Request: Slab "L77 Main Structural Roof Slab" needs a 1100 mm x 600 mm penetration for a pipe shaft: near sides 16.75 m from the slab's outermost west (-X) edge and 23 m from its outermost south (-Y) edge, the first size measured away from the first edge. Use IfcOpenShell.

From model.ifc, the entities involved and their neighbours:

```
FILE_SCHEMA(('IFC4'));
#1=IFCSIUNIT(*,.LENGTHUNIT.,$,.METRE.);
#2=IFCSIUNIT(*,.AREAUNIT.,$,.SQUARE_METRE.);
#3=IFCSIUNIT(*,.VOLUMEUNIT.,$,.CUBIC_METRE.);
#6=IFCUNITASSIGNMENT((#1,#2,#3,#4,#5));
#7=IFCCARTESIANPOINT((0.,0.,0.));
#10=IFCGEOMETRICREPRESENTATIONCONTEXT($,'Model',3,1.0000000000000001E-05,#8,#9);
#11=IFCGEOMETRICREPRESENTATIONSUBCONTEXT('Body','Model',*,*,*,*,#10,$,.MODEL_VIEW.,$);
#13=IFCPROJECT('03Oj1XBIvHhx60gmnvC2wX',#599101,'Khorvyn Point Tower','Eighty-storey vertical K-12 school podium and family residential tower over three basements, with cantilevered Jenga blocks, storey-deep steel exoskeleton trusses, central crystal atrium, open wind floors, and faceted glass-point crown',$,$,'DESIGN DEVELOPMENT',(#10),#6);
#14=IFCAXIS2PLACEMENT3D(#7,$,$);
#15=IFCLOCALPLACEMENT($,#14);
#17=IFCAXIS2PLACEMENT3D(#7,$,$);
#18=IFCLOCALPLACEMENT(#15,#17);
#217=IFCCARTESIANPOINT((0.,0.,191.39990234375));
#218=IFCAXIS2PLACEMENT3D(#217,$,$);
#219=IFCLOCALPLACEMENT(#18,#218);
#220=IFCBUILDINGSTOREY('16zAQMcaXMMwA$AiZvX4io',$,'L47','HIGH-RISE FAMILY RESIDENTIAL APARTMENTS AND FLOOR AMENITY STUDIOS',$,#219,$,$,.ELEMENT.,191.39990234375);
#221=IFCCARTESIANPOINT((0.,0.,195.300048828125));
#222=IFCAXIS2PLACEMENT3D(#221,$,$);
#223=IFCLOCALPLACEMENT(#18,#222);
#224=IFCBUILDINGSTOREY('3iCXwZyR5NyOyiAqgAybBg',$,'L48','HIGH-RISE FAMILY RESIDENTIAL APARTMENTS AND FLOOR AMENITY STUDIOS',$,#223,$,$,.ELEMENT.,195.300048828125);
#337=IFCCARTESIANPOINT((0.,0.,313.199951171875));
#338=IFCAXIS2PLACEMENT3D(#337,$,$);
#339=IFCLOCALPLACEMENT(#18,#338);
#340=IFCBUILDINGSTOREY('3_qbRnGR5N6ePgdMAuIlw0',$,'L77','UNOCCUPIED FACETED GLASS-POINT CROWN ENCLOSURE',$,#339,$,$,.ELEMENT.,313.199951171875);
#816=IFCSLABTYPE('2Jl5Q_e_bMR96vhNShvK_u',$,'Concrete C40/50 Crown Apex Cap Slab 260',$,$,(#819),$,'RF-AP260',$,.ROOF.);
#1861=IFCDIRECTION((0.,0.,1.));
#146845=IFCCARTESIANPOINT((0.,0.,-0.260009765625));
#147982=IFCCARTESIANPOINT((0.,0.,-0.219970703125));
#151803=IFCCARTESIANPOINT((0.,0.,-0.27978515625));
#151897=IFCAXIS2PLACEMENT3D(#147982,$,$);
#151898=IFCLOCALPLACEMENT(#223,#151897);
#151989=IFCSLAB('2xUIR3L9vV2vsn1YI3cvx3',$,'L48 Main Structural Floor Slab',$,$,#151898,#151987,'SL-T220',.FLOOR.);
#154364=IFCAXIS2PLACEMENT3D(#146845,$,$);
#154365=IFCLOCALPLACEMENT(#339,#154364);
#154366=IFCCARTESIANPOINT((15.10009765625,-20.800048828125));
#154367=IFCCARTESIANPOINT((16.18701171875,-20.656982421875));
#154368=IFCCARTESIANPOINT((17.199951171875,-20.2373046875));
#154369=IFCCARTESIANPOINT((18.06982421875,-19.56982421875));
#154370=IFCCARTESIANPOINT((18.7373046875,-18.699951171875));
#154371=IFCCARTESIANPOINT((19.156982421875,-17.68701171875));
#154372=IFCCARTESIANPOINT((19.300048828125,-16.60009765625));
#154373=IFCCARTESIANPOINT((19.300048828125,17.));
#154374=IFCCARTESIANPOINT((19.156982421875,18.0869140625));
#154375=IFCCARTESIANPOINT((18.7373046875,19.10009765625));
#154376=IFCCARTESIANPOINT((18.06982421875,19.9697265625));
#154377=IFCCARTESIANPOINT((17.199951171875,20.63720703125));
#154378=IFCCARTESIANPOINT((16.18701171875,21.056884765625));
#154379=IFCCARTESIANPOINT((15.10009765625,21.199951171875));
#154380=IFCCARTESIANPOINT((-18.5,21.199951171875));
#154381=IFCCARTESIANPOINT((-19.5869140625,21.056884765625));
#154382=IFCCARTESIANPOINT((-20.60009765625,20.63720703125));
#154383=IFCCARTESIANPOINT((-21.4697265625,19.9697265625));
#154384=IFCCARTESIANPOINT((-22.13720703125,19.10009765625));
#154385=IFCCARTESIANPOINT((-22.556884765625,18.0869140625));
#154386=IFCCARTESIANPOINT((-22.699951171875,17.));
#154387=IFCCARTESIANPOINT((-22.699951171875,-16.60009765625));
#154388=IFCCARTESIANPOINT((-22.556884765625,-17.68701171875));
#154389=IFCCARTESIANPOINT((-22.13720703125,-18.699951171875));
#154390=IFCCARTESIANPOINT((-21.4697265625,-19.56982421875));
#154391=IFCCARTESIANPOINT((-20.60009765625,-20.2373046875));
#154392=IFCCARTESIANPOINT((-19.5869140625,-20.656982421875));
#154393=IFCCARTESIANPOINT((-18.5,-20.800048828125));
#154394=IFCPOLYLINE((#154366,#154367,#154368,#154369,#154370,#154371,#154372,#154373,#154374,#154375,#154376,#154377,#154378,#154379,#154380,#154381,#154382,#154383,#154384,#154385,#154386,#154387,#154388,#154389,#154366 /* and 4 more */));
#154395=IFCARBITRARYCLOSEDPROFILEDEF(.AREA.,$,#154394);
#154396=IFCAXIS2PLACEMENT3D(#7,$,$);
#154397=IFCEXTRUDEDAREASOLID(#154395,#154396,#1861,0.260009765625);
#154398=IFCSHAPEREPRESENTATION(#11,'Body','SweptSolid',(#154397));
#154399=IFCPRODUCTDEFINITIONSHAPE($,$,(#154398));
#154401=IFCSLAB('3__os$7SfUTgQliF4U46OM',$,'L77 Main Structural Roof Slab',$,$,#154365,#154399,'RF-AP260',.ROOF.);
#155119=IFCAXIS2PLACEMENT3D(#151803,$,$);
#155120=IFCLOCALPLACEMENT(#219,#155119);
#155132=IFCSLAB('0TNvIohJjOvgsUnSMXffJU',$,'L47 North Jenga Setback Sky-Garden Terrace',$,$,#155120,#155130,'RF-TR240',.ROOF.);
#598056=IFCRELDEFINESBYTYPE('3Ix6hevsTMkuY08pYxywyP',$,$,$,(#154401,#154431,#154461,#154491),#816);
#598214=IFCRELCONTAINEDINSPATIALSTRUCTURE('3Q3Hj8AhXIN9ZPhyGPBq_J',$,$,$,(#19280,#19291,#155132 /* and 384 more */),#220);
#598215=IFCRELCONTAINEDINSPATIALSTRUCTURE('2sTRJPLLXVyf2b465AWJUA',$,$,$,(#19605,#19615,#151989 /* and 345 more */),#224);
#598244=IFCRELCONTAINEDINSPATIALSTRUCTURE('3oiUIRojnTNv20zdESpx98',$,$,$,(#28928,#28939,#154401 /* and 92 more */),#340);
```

```python
import numpy as np
import ifcopenshell
import ifcopenshell.api.feature
import ifcopenshell.api.geometry
import ifcopenshell.api.root
import ifcopenshell.geom
import ifcopenshell.util.placement
import ifcopenshell.util.representation
import ifcopenshell.util.shape
import ifcopenshell.util.unit

model = ifcopenshell.open("model.ifc")
unit_scale = ifcopenshell.util.unit.calculate_unit_scale(model)
settings = ifcopenshell.geom.settings()


def volume(element):
    """Net volume in cubic metres, openings subtracted."""
    shape = ifcopenshell.geom.create_shape(settings, element)
    return ifcopenshell.util.shape.get_volume(shape.geometry)


slab = model.by_guid("3__os$7SfUTgQliF4U46OM")
before = volume(slab)

# Extent in the slab's own axes, in metres. The edges named are its -X and -Y sides.
slab_shape = ifcopenshell.geom.create_shape(settings, slab)
vertices = ifcopenshell.util.shape.get_vertices(slab_shape.geometry)
x_min, y_min, bottom = vertices.min(axis=0)
top = vertices[:, 2].max()

opening = ifcopenshell.api.root.create_entity(model, ifc_class="IfcOpeningElement", name="Pipe shaft opening", predefined_type="OPENING")
context = ifcopenshell.util.representation.get_context(model, "Model", "Body", "MODEL_VIEW")
width, depth = 1.1, 0.6
outline = [(0.0, 0.0), (width, 0.0), (width, depth), (0.0, depth), (0.0, 0.0)]
# Overshoot both faces by 50 mm so the cut is clean.
shape = ifcopenshell.api.geometry.add_slab_representation(
    model, context=context, depth=top - bottom + 0.1, polyline=outline
)
ifcopenshell.api.geometry.assign_representation(model, product=opening, representation=shape)

matrix = ifcopenshell.util.placement.get_local_placement(slab.ObjectPlacement)
matrix[:, 3] = matrix @ np.append(np.array([x_min + 16.75, y_min + 23, bottom - 0.05]) / unit_scale, 1.0)
ifcopenshell.api.geometry.edit_object_placement(model, product=opening, matrix=matrix, is_si=False)
ifcopenshell.api.feature.add_feature(model, feature=opening, element=slab)

after = volume(slab)

print(f"slab volume {before:.3f} -> {after:.3f} m3")

model.write("model_v2.ifc")
```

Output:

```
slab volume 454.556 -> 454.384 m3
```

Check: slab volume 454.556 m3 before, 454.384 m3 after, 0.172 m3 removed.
